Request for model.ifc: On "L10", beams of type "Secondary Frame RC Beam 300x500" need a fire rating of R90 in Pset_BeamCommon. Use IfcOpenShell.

First a look at what the model holds.

```python
import ifcopenshell
import ifcopenshell.util.element

model = ifcopenshell.open("model.ifc")
print(model.schema)
storey = next(s for s in model.by_type("IfcBuildingStorey") if s.Name == "L10")
beams = [e for e in ifcopenshell.util.element.get_decomposition(storey) if e.is_a("IfcBeam")]
seen = {}
for e in beams:
    element_type = ifcopenshell.util.element.get_type(e)
    key = (element_type.Name if element_type != e and element_type else None, ifcopenshell.util.element.get_pset(e, "Pset_BeamCommon", "FireRating"))
    seen[key] = seen.get(key, 0) + 1
for (name, value), count in sorted(seen.items(), key=str):
    print(count, "x", name, "|", value)
```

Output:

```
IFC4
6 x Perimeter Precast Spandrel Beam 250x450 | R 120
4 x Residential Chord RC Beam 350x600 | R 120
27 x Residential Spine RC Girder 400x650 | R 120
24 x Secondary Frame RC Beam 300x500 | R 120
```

```python
import ifcopenshell
import ifcopenshell.api.pset
import ifcopenshell.util.element

model = ifcopenshell.open("model.ifc")

storey = next(s for s in model.by_type("IfcBuildingStorey") if s.Name == "L10")
beams = [e for e in ifcopenshell.util.element.get_decomposition(storey) if e.is_a("IfcBeam")]

count = 0
for e in beams:
    element_type = ifcopenshell.util.element.get_type(e)
    if element_type in (None, e) or element_type.Name != "Secondary Frame RC Beam 300x500":
        continue
    # add_pset returns the element's existing set when there is one.
    pset = ifcopenshell.api.pset.add_pset(model, product=e, name="Pset_BeamCommon")
    ifcopenshell.api.pset.edit_pset(model, pset=pset, properties={"FireRating": "R90"})
    count += 1

print(count, "beams updated")

model.write("model-out.ifc")
```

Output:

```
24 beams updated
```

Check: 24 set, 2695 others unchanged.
